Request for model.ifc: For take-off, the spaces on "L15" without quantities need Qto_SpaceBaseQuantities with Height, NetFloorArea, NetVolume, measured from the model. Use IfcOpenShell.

First a look at what the model holds.

```python
import ifcopenshell
import ifcopenshell.util.element
import ifcopenshell.util.unit

model = ifcopenshell.open("model.ifc")
print(model.schema)
for unit_type in ("LENGTHUNIT", "AREAUNIT", "VOLUMEUNIT"):
    print(unit_type, ifcopenshell.util.unit.calculate_unit_scale(model, unit_type))
storey = next(s for s in model.by_type("IfcBuildingStorey") if s.Name == "L15")
spaces = [e for e in ifcopenshell.util.element.get_decomposition(storey) if e.is_a("IfcSpace")]
for e in sorted(spaces, key=lambda e: e.id()):
    print(e.id(), e.is_a(), e.Name, list(ifcopenshell.util.element.get_psets(e, qtos_only=True)), sep=" | ")
```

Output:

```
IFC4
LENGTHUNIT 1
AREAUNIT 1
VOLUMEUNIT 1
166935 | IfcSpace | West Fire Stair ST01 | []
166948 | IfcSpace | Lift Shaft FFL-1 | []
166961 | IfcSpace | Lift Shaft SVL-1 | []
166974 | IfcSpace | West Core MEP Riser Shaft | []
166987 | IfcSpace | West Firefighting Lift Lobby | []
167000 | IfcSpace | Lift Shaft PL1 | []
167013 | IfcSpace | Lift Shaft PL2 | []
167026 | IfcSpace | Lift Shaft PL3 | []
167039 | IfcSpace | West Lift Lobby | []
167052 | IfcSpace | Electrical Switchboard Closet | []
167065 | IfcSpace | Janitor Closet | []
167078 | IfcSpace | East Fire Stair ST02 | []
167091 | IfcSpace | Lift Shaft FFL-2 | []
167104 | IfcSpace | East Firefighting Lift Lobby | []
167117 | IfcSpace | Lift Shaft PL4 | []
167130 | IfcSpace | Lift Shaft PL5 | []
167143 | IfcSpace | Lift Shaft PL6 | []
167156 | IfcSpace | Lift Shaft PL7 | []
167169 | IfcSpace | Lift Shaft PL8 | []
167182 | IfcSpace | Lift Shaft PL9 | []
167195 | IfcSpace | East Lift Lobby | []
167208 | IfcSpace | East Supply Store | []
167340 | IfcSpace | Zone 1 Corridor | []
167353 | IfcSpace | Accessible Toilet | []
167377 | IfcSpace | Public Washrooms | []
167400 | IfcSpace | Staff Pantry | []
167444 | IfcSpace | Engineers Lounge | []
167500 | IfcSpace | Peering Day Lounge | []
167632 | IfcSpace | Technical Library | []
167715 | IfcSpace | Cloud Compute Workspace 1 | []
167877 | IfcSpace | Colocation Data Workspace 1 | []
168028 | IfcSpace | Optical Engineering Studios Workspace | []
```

```python
import ifcopenshell
import ifcopenshell.api.pset
import ifcopenshell.geom
import ifcopenshell.util.element
import ifcopenshell.util.shape
import ifcopenshell.util.unit

model = ifcopenshell.open("model.ifc")
unit_scale = ifcopenshell.util.unit.calculate_unit_scale(model)
area_scale = ifcopenshell.util.unit.calculate_unit_scale(model, "AREAUNIT")
volume_scale = ifcopenshell.util.unit.calculate_unit_scale(model, "VOLUMEUNIT")
settings = ifcopenshell.geom.settings()

storey = next(s for s in model.by_type("IfcBuildingStorey") if s.Name == "L15")
spaces = [e for e in ifcopenshell.util.element.get_decomposition(storey) if e.is_a("IfcSpace")]

for e in sorted(spaces, key=lambda e: e.id()):
    if ifcopenshell.util.element.get_psets(e, qtos_only=True, should_inherit=False):
        continue
    # Geometry comes back in metres, in the element's own axes.
    shape = ifcopenshell.geom.create_shape(settings, e)
    values = {
        "Height": ifcopenshell.util.shape.get_z(shape.geometry) / unit_scale,
        "NetFloorArea": ifcopenshell.util.shape.get_footprint_area(shape.geometry) / area_scale,
        "NetVolume": ifcopenshell.util.shape.get_volume(shape.geometry) / volume_scale,
    }
    qto = ifcopenshell.api.pset.add_qto(model, product=e, name="Qto_SpaceBaseQuantities")
    ifcopenshell.api.pset.edit_qto(model, qto=qto, properties=values)
    print(e.id(), {k: round(v, 3) for k, v in values.items()})

model.write("model_rev.ifc")
```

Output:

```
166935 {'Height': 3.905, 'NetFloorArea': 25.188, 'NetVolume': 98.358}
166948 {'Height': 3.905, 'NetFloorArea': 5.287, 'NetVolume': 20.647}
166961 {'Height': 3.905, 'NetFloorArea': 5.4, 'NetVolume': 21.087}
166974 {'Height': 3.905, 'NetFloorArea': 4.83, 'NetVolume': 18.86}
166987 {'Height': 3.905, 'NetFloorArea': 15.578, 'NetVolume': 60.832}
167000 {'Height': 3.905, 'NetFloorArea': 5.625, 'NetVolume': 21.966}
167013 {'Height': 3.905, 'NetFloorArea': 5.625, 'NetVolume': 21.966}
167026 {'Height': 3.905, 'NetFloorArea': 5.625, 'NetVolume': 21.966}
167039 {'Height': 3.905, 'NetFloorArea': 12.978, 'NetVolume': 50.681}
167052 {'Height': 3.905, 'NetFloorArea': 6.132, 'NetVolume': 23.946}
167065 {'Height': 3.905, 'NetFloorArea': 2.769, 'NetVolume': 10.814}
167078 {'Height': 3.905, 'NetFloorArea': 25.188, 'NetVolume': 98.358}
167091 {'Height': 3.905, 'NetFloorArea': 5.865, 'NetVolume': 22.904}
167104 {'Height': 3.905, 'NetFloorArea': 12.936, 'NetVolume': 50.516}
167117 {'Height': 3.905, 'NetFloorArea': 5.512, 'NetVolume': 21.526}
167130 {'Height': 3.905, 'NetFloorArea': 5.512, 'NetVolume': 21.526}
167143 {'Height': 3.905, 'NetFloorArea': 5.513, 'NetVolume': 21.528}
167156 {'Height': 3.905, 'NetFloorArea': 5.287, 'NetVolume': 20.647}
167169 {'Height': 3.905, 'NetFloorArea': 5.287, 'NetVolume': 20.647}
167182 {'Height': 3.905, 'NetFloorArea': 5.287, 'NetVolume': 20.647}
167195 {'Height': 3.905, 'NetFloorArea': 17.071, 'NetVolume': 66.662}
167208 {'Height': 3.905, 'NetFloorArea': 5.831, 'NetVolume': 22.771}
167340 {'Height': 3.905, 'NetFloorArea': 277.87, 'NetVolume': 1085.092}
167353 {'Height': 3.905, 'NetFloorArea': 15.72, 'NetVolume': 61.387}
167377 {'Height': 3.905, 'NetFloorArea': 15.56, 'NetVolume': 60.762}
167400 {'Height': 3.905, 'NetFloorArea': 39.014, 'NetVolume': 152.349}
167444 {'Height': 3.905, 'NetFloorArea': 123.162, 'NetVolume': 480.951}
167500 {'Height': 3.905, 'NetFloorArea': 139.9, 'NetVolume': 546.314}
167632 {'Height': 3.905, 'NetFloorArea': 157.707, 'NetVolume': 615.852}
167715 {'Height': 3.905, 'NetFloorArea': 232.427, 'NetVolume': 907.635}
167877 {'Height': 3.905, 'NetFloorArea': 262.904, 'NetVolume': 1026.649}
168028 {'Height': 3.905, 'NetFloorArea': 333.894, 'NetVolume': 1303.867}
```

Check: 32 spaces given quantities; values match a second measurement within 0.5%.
